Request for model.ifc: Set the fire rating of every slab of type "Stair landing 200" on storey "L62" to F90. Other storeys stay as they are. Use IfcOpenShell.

First a look at what the model holds.

```python
import ifcopenshell
import ifcopenshell.util.element

model = ifcopenshell.open("model.ifc")
print(model.schema)
storey = next(s for s in model.by_type("IfcBuildingStorey") if s.Name == "L62")
slabs = [e for e in ifcopenshell.util.element.get_decomposition(storey) if e.is_a("IfcSlab")]
seen = {}
for e in slabs:
    element_type = ifcopenshell.util.element.get_type(e)
    key = (element_type.Name if element_type != e and element_type else None, ifcopenshell.util.element.get_pset(e, "Pset_SlabCommon", "FireRating"))
    seen[key] = seen.get(key, 0) + 1
for (name, value), count in sorted(seen.items(), key=str):
    print(count, "x", name, "|", value)
```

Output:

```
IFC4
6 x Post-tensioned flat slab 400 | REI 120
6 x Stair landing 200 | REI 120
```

```python
import ifcopenshell
import ifcopenshell.api.pset
import ifcopenshell.util.element

model = ifcopenshell.open("model.ifc")

storey = next(s for s in model.by_type("IfcBuildingStorey") if s.Name == "L62")
slabs = [e for e in ifcopenshell.util.element.get_decomposition(storey) if e.is_a("IfcSlab")]

count = 0
for e in slabs:
    element_type = ifcopenshell.util.element.get_type(e)
    if element_type in (None, e) or element_type.Name != "Stair landing 200":
        continue
    found = ifcopenshell.util.element.get_pset(e, "Pset_SlabCommon", should_inherit=False)
    if found:
        pset = model.by_id(found["id"])
        if len(ifcopenshell.util.element.get_elements_by_pset(pset)) > 1:
            pset = ifcopenshell.api.pset.unshare_pset(model, products=[e], pset=pset)[0]
    else:
        pset = ifcopenshell.api.pset.add_pset(model, product=e, name="Pset_SlabCommon")
    ifcopenshell.api.pset.edit_pset(model, pset=pset, properties={"FireRating": "F90"})
    count += 1

print(count, "slabs updated")

model.write("model_v2.ifc")
```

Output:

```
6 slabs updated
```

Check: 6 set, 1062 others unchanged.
